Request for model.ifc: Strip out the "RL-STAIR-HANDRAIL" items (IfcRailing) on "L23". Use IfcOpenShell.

First a look at what the model holds.

```python
import ifcopenshell
import ifcopenshell.util.element

model = ifcopenshell.open("model.ifc")
print(model.schema)
storey = next(s for s in model.by_type("IfcBuildingStorey") if s.Name == "L23")
railings = [e for e in ifcopenshell.util.element.get_decomposition(storey) if e.is_a("IfcRailing")]
seen = {}
for e in railings:
    element_type = ifcopenshell.util.element.get_type(e)
    name = element_type.Name if element_type not in (None, e) else None
    seen[name] = seen.get(name, 0) + 1
for name, count in sorted(seen.items(), key=str):
    print(count, "x", name)
```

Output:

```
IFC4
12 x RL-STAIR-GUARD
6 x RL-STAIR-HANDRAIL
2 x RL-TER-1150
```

```python
import ifcopenshell
import ifcopenshell.api.root
import ifcopenshell.util.element

model = ifcopenshell.open("model.ifc")

storey = next(s for s in model.by_type("IfcBuildingStorey") if s.Name == "L23")
railings = [e for e in ifcopenshell.util.element.get_decomposition(storey) if e.is_a("IfcRailing")]
targets = [e for e in railings if (t := ifcopenshell.util.element.get_type(e)) not in (None, e) and t.Name == "RL-STAIR-HANDRAIL"]

for e in targets:
    ifcopenshell.api.root.remove_product(model, product=e)
print(len(targets), "removed")

model.write("model_v2.ifc")
```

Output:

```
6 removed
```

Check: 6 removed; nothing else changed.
